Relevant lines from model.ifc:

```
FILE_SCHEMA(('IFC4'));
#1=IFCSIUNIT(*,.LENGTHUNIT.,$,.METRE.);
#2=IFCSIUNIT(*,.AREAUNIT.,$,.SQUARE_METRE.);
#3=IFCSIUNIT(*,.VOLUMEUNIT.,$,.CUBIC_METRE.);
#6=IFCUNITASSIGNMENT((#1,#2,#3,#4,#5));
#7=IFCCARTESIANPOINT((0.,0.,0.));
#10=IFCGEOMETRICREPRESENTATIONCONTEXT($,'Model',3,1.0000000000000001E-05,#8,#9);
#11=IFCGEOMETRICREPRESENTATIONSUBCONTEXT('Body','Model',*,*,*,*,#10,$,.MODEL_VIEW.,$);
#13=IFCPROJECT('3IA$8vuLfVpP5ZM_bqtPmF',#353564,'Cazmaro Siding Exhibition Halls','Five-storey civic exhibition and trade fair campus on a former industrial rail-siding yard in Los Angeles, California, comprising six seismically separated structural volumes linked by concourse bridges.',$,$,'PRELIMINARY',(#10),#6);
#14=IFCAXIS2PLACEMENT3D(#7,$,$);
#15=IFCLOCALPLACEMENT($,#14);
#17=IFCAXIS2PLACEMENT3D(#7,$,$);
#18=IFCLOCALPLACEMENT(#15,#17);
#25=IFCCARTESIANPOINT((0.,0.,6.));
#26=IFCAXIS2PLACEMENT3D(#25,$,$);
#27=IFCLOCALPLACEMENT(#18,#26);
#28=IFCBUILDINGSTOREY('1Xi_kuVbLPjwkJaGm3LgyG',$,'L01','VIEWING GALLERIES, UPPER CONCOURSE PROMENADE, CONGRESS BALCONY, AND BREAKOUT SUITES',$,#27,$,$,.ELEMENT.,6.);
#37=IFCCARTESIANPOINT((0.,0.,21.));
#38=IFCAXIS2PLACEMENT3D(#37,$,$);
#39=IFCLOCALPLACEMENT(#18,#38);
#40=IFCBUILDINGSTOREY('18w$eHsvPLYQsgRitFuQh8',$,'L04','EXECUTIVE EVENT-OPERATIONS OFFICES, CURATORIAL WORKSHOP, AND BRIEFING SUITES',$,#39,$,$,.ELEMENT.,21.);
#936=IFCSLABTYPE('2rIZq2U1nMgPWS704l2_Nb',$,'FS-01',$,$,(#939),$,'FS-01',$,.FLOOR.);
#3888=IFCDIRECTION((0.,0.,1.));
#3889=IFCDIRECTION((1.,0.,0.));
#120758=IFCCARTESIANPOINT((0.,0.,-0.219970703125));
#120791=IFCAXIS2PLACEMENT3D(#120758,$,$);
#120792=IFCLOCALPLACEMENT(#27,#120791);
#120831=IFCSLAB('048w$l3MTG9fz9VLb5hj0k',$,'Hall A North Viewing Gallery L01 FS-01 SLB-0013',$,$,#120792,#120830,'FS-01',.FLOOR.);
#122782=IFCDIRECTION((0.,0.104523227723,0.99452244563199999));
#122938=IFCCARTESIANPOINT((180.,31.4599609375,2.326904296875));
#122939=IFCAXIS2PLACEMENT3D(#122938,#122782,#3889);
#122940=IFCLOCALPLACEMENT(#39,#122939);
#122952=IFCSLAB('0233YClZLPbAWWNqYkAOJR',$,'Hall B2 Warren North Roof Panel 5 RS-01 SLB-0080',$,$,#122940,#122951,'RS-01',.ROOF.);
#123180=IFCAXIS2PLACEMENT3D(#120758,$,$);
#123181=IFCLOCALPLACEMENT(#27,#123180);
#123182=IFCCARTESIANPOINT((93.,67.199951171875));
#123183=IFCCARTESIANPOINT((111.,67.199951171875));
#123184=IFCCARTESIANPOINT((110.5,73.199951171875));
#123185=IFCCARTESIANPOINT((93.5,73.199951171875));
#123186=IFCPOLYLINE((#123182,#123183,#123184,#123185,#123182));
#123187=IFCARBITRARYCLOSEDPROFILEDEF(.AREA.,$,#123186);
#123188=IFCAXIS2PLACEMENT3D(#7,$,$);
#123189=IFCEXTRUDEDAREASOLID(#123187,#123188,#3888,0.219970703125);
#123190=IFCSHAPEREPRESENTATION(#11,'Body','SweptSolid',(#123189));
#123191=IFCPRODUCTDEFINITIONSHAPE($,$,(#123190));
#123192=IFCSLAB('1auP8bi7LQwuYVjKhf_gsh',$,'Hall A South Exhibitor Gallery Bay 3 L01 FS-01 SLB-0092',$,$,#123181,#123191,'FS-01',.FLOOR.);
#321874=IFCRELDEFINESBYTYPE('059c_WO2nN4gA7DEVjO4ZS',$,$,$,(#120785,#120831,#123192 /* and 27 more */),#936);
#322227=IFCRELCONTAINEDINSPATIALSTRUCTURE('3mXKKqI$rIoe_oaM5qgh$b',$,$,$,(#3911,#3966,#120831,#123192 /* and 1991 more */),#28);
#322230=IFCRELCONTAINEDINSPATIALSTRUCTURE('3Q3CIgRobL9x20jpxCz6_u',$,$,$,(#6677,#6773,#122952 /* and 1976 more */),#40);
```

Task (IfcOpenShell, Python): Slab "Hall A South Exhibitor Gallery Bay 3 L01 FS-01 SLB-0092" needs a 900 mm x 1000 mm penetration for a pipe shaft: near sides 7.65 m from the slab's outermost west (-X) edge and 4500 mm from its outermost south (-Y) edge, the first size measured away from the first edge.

```python
import numpy as np
import ifcopenshell
import ifcopenshell.api.feature
import ifcopenshell.api.geometry
import ifcopenshell.api.root
import ifcopenshell.geom
import ifcopenshell.util.placement
import ifcopenshell.util.representation
import ifcopenshell.util.shape
import ifcopenshell.util.unit

model = ifcopenshell.open("model.ifc")
unit_scale = ifcopenshell.util.unit.calculate_unit_scale(model)
settings = ifcopenshell.geom.settings()


def volume(element):
    """Net volume in cubic metres, openings subtracted."""
    shape = ifcopenshell.geom.create_shape(settings, element)
    return ifcopenshell.util.shape.get_volume(shape.geometry)


slab = model.by_id(123192)
before = volume(slab)

# Extent in the slab's own axes, in metres. The edges named are its -X and -Y sides.
slab_shape = ifcopenshell.geom.create_shape(settings, slab)
vertices = ifcopenshell.util.shape.get_vertices(slab_shape.geometry)
x_min, y_min, bottom = vertices.min(axis=0)
top = vertices[:, 2].max()

opening = ifcopenshell.api.root.create_entity(model, ifc_class="IfcOpeningElement", name="Pipe shaft opening", predefined_type="OPENING")
context = ifcopenshell.util.representation.get_context(model, "Model", "Body", "MODEL_VIEW")
width, depth = 0.9, 1
outline = [(0.0, 0.0), (width, 0.0), (width, depth), (0.0, depth), (0.0, 0.0)]
# Overshoot both faces by 50 mm so the cut is clean.
shape = ifcopenshell.api.geometry.add_slab_representation(
    model, context=context, depth=top - bottom + 0.1, polyline=outline
)
ifcopenshell.api.geometry.assign_representation(model, product=opening, representation=shape)

matrix = ifcopenshell.util.placement.get_local_placement(slab.ObjectPlacement)
matrix[:, 3] = matrix @ np.append(np.array([x_min + 7.65, y_min + 4.5, bottom - 0.05]) / unit_scale, 1.0)
ifcopenshell.api.geometry.edit_object_placement(model, product=opening, matrix=matrix, is_si=False)
ifcopenshell.api.feature.add_feature(model, feature=opening, element=slab)

after = volume(slab)

print(f"slab volume {before:.3f} -> {after:.3f} m3")

model.write("model-out.ifc")
```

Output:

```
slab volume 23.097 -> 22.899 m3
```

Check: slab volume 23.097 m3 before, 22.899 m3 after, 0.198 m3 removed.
